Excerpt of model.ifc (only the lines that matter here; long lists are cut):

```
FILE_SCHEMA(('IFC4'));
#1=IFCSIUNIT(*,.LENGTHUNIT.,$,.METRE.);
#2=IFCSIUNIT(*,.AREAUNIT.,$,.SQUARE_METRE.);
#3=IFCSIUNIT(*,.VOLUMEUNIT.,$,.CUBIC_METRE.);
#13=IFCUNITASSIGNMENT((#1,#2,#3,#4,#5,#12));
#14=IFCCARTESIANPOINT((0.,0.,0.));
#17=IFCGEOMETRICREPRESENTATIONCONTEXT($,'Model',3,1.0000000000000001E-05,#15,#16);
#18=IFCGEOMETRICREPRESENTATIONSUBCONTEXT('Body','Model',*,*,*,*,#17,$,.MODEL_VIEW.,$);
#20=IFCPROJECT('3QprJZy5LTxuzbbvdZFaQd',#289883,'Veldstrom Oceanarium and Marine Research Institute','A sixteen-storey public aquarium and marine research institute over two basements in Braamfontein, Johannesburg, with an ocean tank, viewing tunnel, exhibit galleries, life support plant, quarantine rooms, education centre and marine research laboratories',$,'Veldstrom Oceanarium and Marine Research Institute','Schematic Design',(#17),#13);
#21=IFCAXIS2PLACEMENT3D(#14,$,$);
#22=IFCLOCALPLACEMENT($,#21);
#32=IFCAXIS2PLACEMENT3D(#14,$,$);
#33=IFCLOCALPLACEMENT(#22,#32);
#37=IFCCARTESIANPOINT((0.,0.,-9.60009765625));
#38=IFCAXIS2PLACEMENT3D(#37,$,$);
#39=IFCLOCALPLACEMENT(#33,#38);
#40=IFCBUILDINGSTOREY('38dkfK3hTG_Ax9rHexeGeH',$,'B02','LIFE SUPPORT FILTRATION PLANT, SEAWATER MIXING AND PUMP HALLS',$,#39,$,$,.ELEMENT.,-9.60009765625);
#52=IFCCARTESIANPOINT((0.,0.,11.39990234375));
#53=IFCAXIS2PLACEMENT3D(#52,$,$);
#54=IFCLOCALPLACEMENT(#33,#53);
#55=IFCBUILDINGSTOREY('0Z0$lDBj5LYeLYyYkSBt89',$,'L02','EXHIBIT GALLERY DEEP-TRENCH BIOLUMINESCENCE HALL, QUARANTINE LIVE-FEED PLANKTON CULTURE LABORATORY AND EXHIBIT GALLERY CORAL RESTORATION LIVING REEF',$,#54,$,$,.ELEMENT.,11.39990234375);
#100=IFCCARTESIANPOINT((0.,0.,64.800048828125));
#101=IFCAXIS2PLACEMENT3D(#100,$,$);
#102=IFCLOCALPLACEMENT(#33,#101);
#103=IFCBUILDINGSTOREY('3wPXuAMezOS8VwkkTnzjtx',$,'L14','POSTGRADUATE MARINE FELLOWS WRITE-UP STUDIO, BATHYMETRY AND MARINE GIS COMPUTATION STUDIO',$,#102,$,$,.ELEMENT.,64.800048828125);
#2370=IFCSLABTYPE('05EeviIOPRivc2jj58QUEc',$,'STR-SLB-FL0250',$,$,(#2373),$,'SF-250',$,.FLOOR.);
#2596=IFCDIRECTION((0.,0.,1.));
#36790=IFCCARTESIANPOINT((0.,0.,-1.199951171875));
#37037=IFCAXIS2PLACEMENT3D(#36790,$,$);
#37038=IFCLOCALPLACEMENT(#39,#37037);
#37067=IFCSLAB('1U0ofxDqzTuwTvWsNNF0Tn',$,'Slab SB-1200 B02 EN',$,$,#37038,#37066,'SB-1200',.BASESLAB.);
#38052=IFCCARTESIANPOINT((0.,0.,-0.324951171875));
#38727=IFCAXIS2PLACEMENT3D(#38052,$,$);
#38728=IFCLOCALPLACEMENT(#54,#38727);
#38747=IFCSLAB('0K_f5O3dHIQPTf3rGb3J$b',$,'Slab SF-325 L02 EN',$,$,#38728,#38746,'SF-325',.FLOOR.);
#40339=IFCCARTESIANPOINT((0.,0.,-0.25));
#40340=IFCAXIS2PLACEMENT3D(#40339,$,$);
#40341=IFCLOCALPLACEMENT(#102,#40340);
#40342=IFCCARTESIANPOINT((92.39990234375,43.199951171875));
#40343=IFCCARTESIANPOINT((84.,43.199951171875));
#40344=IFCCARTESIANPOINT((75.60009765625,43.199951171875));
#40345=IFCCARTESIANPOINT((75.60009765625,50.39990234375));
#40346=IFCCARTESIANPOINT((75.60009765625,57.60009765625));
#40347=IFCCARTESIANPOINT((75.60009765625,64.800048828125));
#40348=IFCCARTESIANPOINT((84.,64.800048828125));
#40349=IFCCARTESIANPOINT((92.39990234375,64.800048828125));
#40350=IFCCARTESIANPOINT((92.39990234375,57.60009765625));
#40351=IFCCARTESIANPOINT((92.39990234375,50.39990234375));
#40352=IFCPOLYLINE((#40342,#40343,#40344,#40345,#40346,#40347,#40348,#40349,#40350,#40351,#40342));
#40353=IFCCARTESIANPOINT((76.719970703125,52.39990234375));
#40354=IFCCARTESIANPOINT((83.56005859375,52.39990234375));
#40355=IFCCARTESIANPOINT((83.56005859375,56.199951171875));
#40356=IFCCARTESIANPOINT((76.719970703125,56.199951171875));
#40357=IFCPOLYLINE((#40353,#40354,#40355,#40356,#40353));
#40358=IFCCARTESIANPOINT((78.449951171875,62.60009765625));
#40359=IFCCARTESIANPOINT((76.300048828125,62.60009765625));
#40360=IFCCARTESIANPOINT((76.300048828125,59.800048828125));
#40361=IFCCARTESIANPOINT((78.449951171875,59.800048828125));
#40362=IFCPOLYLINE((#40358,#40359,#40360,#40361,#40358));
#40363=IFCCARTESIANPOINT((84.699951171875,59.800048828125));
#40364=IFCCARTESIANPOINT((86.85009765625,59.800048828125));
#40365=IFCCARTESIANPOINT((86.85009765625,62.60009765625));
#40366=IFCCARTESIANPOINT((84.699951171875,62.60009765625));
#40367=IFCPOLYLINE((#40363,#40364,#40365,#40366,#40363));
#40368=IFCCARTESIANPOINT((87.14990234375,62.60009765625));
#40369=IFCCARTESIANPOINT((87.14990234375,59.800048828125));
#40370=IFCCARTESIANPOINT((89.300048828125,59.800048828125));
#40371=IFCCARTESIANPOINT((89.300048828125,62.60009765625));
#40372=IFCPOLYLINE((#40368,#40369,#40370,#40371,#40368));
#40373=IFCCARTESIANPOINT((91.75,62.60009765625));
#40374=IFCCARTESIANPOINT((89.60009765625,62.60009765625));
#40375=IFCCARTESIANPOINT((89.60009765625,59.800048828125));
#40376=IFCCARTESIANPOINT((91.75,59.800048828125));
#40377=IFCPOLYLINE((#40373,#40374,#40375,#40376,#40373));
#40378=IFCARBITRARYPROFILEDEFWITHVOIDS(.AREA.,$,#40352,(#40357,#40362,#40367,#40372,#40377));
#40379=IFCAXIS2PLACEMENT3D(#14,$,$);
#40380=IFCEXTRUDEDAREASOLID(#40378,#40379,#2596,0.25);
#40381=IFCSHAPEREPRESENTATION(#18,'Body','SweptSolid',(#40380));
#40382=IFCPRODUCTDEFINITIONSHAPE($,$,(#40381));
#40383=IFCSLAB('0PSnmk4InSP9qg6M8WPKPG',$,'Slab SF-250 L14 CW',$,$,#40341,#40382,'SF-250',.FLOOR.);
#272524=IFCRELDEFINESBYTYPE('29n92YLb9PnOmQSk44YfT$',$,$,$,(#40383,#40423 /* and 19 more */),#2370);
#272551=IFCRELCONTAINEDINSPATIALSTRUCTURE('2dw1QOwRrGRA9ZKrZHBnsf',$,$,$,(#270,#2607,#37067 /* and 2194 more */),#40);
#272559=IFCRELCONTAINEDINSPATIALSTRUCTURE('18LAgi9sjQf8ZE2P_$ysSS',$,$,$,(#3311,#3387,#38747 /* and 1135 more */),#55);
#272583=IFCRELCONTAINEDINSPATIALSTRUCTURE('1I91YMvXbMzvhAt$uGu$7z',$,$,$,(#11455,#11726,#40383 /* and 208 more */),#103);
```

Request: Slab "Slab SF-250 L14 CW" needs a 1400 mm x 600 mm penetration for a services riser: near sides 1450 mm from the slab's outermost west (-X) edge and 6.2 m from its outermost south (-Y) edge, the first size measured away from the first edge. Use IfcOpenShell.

```python
import numpy as np
import ifcopenshell
import ifcopenshell.api.feature
import ifcopenshell.api.geometry
import ifcopenshell.api.root
import ifcopenshell.geom
import ifcopenshell.util.placement
import ifcopenshell.util.representation
import ifcopenshell.util.shape
import ifcopenshell.util.unit

model = ifcopenshell.open("model.ifc")
unit_scale = ifcopenshell.util.unit.calculate_unit_scale(model)
settings = ifcopenshell.geom.settings()


def volume(element):
    """Net volume in cubic metres, openings subtracted."""
    shape = ifcopenshell.geom.create_shape(settings, element)
    return ifcopenshell.util.shape.get_volume(shape.geometry)


slab = model.by_guid("0PSnmk4InSP9qg6M8WPKPG")
before = volume(slab)

# Extent in the slab's own axes, in metres. The edges named are its -X and -Y sides.
slab_shape = ifcopenshell.geom.create_shape(settings, slab)
vertices = ifcopenshell.util.shape.get_vertices(slab_shape.geometry)
x_min, y_min, bottom = vertices.min(axis=0)
top = vertices[:, 2].max()

opening = ifcopenshell.api.root.create_entity(model, ifc_class="IfcOpeningElement", name="Services riser opening", predefined_type="OPENING")
context = ifcopenshell.util.representation.get_context(model, "Model", "Body", "MODEL_VIEW")
width, depth = 1.4, 0.6
outline = [(0.0, 0.0), (width, 0.0), (width, depth), (0.0, depth), (0.0, 0.0)]
# Overshoot both faces by 50 mm so the cut is clean.
shape = ifcopenshell.api.geometry.add_slab_representation(
    model, context=context, depth=top - bottom + 0.1, polyline=outline
)
ifcopenshell.api.geometry.assign_representation(model, product=opening, representation=shape)

matrix = ifcopenshell.util.placement.get_local_placement(slab.ObjectPlacement)
matrix[:, 3] = matrix @ np.append(np.array([x_min + 1.45, y_min + 6.2, bottom - 0.05]) / unit_scale, 1.0)
ifcopenshell.api.geometry.edit_object_placement(model, product=opening, matrix=matrix, is_si=False)
ifcopenshell.api.feature.add_feature(model, feature=opening, element=slab)

after = volume(slab)

print(f"slab volume {before:.3f} -> {after:.3f} m3")

model.write("model-out.ifc")
```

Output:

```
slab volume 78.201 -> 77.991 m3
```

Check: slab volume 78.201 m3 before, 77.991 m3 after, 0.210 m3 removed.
